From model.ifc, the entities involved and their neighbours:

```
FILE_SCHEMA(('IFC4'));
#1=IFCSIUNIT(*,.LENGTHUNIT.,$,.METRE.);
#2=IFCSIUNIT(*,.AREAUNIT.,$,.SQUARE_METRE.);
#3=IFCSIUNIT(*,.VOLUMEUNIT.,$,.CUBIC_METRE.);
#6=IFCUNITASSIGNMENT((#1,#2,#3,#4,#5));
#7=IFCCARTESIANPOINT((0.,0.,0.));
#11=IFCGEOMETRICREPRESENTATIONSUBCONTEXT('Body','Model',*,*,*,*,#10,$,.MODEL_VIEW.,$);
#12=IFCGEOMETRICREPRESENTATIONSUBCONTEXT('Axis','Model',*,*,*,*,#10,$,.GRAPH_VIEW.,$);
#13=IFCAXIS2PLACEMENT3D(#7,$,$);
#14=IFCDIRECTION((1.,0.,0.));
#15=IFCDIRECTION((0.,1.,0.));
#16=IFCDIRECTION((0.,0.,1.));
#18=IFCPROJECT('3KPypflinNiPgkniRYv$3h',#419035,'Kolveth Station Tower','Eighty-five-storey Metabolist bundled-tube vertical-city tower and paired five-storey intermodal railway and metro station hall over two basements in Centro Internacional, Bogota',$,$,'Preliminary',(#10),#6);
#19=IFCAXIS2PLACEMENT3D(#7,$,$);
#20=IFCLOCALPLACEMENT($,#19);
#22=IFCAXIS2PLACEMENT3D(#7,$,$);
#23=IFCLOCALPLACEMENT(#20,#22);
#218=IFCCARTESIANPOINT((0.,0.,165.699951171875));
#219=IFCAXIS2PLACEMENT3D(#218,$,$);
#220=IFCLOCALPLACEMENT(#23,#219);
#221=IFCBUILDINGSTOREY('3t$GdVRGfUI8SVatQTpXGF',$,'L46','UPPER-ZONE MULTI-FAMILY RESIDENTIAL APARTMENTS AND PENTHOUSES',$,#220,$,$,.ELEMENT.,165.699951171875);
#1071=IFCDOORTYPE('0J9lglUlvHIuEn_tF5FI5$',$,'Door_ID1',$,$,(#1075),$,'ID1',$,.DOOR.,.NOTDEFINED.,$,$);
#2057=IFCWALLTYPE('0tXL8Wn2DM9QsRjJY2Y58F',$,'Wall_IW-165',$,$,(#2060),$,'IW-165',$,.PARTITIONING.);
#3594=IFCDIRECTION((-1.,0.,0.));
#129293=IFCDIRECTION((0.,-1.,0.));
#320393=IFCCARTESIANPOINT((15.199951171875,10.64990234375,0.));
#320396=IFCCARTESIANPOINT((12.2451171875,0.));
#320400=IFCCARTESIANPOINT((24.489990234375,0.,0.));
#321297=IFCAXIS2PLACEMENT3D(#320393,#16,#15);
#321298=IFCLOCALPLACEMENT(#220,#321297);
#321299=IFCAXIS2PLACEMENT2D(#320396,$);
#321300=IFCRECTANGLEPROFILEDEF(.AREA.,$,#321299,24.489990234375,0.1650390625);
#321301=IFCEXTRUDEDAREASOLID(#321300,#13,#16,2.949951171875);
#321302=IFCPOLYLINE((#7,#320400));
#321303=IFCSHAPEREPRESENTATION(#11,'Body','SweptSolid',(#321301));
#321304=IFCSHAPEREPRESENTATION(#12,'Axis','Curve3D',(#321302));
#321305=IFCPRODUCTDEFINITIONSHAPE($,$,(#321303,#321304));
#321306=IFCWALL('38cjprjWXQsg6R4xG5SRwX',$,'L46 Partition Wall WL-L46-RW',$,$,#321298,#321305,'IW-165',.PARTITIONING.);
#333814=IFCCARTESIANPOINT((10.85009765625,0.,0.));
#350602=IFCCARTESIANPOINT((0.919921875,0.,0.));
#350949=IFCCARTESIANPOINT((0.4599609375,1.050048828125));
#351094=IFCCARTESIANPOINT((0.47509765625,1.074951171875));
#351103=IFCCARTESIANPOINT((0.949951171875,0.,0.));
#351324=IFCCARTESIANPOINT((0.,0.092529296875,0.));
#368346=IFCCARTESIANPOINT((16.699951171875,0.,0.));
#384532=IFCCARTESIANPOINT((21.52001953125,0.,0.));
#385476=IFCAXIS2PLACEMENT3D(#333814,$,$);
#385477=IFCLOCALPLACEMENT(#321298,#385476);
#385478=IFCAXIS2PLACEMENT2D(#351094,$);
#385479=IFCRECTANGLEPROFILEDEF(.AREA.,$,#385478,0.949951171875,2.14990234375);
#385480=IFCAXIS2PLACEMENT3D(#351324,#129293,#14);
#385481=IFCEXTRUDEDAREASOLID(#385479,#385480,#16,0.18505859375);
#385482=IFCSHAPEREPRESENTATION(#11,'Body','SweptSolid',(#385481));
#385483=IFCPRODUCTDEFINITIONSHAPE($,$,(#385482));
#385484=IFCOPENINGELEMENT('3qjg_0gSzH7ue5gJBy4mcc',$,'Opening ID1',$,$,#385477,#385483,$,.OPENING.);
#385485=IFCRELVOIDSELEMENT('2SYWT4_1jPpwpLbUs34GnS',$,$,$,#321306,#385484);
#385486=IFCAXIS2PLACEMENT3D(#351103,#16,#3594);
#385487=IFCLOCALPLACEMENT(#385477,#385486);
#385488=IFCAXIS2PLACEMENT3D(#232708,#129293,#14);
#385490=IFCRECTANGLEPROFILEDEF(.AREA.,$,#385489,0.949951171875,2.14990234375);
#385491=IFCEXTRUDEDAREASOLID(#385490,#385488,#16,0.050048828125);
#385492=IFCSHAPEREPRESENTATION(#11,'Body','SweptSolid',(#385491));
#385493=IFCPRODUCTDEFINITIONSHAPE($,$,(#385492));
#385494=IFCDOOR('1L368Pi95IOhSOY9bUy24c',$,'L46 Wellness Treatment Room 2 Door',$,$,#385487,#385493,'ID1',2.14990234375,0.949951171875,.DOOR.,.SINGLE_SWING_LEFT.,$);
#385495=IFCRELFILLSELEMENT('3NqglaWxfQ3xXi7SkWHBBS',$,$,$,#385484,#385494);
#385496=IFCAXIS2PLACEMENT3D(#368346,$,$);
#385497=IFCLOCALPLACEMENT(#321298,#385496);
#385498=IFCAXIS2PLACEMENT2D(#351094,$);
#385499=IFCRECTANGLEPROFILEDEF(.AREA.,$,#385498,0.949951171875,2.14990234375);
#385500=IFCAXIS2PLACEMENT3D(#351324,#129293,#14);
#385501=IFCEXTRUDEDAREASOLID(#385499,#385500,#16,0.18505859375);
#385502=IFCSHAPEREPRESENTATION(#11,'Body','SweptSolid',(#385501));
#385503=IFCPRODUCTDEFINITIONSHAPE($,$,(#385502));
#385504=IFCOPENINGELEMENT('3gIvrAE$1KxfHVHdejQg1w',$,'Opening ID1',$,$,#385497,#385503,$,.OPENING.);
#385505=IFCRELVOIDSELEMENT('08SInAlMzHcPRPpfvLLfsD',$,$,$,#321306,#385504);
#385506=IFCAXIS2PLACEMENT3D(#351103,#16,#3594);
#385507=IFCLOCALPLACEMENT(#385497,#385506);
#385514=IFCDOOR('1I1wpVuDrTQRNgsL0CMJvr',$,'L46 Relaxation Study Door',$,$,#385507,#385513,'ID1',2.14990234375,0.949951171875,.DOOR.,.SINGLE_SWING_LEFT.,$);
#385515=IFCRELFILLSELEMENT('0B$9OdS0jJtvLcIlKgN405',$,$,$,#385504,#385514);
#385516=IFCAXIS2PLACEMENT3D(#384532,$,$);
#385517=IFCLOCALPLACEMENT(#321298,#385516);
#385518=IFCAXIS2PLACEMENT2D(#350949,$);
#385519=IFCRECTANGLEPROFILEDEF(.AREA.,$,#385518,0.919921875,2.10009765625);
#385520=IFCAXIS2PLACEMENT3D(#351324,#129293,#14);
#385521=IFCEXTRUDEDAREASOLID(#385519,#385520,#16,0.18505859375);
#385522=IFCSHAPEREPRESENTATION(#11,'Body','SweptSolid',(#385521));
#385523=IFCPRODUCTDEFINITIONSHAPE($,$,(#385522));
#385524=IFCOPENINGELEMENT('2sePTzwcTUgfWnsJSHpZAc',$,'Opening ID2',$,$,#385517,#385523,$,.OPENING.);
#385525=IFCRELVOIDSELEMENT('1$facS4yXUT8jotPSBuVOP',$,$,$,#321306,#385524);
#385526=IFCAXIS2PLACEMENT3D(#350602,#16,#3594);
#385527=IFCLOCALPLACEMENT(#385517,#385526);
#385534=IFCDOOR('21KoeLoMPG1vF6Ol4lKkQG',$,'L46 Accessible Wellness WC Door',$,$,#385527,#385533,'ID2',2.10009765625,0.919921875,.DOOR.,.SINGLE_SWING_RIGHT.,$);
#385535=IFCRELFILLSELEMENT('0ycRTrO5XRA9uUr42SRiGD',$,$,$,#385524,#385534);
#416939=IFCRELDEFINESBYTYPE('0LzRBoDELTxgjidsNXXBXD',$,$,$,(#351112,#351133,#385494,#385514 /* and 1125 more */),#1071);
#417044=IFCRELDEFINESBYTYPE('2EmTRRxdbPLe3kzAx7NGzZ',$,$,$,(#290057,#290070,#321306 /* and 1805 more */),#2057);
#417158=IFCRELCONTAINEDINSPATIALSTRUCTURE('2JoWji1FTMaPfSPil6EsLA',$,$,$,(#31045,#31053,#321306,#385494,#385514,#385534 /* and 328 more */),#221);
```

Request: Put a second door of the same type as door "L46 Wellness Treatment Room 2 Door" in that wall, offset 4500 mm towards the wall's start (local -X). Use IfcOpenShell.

```python
import ifcopenshell
import ifcopenshell.api.feature
import ifcopenshell.api.geometry
import ifcopenshell.api.root
import ifcopenshell.geom
import ifcopenshell.util.element
import ifcopenshell.util.placement
import ifcopenshell.util.shape

model = ifcopenshell.open("model.ifc")
settings = ifcopenshell.geom.settings()


def volume(element):
    """Net volume in cubic metres, openings subtracted."""
    shape = ifcopenshell.geom.create_shape(settings, element)
    return ifcopenshell.util.shape.get_volume(shape.geometry)


door = model.by_guid("1L368Pi95IOhSOY9bUy24c")
opening = door.FillsVoids[0].RelatingOpeningElement
wall = opening.VoidsElements[0].RelatingBuildingElement
before = volume(wall)
shift = ifcopenshell.util.placement.get_local_placement(wall.ObjectPlacement)[:3, 0] * -4.5

# copy_class copies the void relationship, type, container and properties, but no geometry.
new_opening = ifcopenshell.api.root.copy_class(model, product=opening)
new_opening.Representation = ifcopenshell.util.element.copy_deep(
    model, opening.Representation, exclude=["IfcGeometricRepresentationContext", "IfcRepresentationMap"]
)
new_door = ifcopenshell.api.root.copy_class(model, product=door)
new_door.Representation = ifcopenshell.util.element.copy_deep(
    model, door.Representation, exclude=["IfcGeometricRepresentationContext", "IfcRepresentationMap"]
)
new_door.Tag = None
ifcopenshell.api.feature.add_filling(model, opening=new_opening, element=new_door)

for old, new in ((opening, new_opening), (door, new_door)):
    matrix = ifcopenshell.util.placement.get_local_placement(old.ObjectPlacement)
    matrix[:3, 3] += shift
    ifcopenshell.api.geometry.edit_object_placement(model, product=new, matrix=matrix, is_si=False)

after = volume(wall)

print(f"wall volume {before:.3f} -> {after:.3f} m3")

model.write("model_v2.ifc")
```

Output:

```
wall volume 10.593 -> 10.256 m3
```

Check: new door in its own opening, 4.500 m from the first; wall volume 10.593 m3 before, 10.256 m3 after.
